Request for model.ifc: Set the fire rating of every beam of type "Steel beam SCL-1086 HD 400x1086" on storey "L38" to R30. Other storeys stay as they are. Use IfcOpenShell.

First a look at what the model holds.

```python
import ifcopenshell
import ifcopenshell.util.element

model = ifcopenshell.open("model.ifc")
print(model.schema)
storey = next(s for s in model.by_type("IfcBuildingStorey") if s.Name == "L38")
beams = [e for e in ifcopenshell.util.element.get_decomposition(storey) if e.is_a("IfcBeam")]
seen = {}
for e in beams:
    element_type = ifcopenshell.util.element.get_type(e)
    key = (element_type.Name if element_type != e and element_type else None, ifcopenshell.util.element.get_pset(e, "Pset_BeamCommon", "FireRating"))
    seen[key] = seen.get(key, 0) + 1
for (name, value), count in sorted(seen.items(), key=str):
    print(count, "x", name, "|", value)
```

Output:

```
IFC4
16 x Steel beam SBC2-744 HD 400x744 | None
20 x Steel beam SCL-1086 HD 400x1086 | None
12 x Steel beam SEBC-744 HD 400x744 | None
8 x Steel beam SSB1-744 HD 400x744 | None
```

```python
import ifcopenshell
import ifcopenshell.api.pset
import ifcopenshell.util.element

model = ifcopenshell.open("model.ifc")

storey = next(s for s in model.by_type("IfcBuildingStorey") if s.Name == "L38")
beams = [e for e in ifcopenshell.util.element.get_decomposition(storey) if e.is_a("IfcBeam")]

count = 0
for e in beams:
    element_type = ifcopenshell.util.element.get_type(e)
    if element_type in (None, e) or element_type.Name != "Steel beam SCL-1086 HD 400x1086":
        continue
    found = ifcopenshell.util.element.get_pset(e, "Pset_BeamCommon", should_inherit=False)
    if found:
        pset = model.by_id(found["id"])
        if len(ifcopenshell.util.element.get_elements_by_pset(pset)) > 1:
            pset = ifcopenshell.api.pset.unshare_pset(model, products=[e], pset=pset)[0]
    else:
        pset = ifcopenshell.api.pset.add_pset(model, product=e, name="Pset_BeamCommon")
    ifcopenshell.api.pset.edit_pset(model, pset=pset, properties={"FireRating": "R30"})
    count += 1

print(count, "beams updated")

model.write("model_updated.ifc")
```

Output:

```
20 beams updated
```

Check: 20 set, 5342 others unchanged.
